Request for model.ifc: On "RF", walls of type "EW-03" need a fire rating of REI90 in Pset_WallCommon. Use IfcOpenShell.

First a look at what the model holds.

```python
import ifcopenshell
import ifcopenshell.util.element

model = ifcopenshell.open("model.ifc")
print(model.schema)
storey = next(s for s in model.by_type("IfcBuildingStorey") if s.Name == "RF")
walls = [e for e in ifcopenshell.util.element.get_decomposition(storey) if e.is_a("IfcWall")]
seen = {}
for e in walls:
    element_type = ifcopenshell.util.element.get_type(e)
    key = (element_type.Name if element_type != e and element_type else None, ifcopenshell.util.element.get_pset(e, "Pset_WallCommon", "FireRating"))
    seen[key] = seen.get(key, 0) + 1
for (name, value), count in sorted(seen.items(), key=str):
    print(count, "x", name, "|", value)
```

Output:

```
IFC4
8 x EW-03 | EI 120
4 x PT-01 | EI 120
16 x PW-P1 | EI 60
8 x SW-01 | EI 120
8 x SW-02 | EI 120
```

```python
import ifcopenshell
import ifcopenshell.api.pset
import ifcopenshell.util.element

model = ifcopenshell.open("model.ifc")

storey = next(s for s in model.by_type("IfcBuildingStorey") if s.Name == "RF")
walls = [e for e in ifcopenshell.util.element.get_decomposition(storey) if e.is_a("IfcWall")]

count = 0
for e in walls:
    element_type = ifcopenshell.util.element.get_type(e)
    if element_type in (None, e) or element_type.Name != "EW-03":
        continue
    # add_pset returns the element's existing set when there is one.
    pset = ifcopenshell.api.pset.add_pset(model, product=e, name="Pset_WallCommon")
    ifcopenshell.api.pset.edit_pset(model, pset=pset, properties={"FireRating": "REI90"})
    count += 1

print(count, "walls updated")

model.write("model-out.ifc")
```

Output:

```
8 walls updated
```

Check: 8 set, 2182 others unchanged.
